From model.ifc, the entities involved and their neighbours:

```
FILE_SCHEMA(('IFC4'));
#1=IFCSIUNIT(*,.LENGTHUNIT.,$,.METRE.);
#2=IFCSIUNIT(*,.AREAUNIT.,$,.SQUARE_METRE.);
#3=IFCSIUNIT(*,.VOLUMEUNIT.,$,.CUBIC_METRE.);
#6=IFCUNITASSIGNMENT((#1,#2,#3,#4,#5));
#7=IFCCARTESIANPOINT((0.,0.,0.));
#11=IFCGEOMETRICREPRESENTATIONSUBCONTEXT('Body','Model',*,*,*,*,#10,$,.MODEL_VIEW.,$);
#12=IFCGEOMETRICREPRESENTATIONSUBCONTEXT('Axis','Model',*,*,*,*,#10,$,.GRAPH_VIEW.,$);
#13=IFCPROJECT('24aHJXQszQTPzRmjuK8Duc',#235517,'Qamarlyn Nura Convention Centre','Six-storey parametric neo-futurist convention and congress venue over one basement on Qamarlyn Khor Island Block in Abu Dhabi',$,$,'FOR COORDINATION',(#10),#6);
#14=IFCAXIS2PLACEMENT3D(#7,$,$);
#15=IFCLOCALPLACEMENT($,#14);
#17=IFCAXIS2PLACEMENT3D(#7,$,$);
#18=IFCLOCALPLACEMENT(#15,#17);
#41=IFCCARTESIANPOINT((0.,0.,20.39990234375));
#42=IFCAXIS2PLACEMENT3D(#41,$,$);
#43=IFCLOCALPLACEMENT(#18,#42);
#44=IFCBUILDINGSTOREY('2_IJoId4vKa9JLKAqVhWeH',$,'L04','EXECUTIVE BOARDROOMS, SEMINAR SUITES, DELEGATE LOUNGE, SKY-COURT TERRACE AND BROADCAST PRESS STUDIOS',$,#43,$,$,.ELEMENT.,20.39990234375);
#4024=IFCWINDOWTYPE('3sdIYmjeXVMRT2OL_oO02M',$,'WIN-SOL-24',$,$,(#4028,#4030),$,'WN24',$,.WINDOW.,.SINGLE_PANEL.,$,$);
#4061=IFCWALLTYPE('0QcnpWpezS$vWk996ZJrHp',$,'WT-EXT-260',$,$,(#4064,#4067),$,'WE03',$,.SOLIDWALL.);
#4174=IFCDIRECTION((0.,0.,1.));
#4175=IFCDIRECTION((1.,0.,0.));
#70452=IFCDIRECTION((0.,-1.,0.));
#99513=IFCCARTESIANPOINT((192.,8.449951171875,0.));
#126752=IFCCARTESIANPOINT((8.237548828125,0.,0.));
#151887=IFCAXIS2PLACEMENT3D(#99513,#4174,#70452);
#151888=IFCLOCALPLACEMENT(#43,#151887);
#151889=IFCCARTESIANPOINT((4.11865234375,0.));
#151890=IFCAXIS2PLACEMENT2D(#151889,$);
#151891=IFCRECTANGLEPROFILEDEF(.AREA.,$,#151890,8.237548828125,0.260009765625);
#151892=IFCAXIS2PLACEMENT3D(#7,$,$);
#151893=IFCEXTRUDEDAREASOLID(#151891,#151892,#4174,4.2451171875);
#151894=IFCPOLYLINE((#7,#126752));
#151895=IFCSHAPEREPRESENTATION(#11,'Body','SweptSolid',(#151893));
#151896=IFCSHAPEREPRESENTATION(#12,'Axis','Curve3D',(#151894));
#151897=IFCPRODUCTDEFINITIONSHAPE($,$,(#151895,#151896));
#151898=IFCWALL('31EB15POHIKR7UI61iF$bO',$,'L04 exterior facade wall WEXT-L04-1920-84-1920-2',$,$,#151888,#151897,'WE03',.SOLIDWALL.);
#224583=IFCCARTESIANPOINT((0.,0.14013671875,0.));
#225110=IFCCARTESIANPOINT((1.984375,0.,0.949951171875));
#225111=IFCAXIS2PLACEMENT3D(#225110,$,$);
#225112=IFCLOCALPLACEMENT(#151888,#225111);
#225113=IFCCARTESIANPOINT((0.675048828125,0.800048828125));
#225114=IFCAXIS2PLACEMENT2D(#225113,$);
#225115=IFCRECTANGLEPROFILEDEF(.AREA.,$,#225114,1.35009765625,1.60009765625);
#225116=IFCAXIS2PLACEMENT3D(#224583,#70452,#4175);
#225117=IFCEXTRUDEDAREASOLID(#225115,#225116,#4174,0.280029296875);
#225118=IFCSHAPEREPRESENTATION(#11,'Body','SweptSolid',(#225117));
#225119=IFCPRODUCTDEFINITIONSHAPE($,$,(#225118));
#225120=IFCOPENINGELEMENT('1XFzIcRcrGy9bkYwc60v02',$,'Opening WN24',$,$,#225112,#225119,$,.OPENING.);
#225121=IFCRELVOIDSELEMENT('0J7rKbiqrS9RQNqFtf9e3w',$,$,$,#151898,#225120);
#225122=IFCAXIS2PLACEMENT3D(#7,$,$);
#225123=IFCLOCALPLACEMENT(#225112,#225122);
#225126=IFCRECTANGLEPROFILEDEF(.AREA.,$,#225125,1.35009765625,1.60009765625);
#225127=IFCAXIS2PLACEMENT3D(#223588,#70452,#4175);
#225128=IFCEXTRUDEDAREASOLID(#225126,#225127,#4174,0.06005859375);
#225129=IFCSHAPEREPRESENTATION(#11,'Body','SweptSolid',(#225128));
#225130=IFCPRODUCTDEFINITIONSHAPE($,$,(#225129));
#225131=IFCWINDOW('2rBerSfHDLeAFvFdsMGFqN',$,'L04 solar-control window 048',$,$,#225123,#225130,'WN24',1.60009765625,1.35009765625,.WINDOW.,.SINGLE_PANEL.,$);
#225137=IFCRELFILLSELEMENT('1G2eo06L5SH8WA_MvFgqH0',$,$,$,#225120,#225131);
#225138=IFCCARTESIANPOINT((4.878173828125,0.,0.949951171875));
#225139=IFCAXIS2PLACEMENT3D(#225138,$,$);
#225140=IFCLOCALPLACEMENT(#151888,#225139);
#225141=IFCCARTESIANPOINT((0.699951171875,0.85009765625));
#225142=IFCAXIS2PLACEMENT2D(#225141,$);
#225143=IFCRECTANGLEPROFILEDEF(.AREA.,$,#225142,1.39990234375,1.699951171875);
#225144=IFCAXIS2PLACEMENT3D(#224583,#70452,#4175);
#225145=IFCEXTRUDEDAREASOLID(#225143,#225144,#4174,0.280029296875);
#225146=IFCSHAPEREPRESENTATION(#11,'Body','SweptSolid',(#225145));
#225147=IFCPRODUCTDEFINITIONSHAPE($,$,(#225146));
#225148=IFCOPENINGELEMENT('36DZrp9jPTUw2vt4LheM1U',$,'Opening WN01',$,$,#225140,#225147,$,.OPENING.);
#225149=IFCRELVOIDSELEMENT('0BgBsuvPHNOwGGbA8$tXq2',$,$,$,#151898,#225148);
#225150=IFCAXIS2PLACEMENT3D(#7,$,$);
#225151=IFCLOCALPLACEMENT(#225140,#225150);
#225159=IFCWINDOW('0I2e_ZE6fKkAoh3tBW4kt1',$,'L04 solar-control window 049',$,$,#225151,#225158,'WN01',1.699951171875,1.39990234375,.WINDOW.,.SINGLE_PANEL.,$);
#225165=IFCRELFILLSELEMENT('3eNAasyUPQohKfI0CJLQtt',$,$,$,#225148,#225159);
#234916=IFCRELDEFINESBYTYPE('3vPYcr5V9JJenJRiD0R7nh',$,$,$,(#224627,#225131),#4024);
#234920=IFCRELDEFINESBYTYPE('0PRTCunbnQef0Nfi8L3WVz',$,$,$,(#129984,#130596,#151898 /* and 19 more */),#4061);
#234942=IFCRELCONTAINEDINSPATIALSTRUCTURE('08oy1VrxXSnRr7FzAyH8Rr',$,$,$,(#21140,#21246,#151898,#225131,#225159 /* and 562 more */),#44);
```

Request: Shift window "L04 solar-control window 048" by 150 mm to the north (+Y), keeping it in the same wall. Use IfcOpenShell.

```python
import ifcopenshell
import ifcopenshell.api.geometry
import ifcopenshell.util.placement
import ifcopenshell.util.unit

model = ifcopenshell.open("model.ifc")
unit_scale = ifcopenshell.util.unit.calculate_unit_scale(model)

window = model.by_guid("2rBerSfHDLeAFvFdsMGFqN")
opening = window.FillsVoids[0].RelatingOpeningElement
wall = opening.VoidsElements[0].RelatingBuildingElement

wall_matrix = ifcopenshell.util.placement.get_local_placement(wall.ObjectPlacement)
shift = wall_matrix[:3, 0] * -0.15 / unit_scale
before = ifcopenshell.util.placement.get_local_placement(window.ObjectPlacement)[:3, 3].copy()

# The window is placed relative to its opening, so it follows when the opening moves.
matrix = ifcopenshell.util.placement.get_local_placement(opening.ObjectPlacement)
matrix[:3, 3] += shift
ifcopenshell.api.geometry.edit_object_placement(
    model, product=opening, matrix=matrix, is_si=False, should_transform_children=True
)

after = ifcopenshell.util.placement.get_local_placement(window.ObjectPlacement)[:3, 3]
print("window moved by", (after - before).round(3) + 0.0)

model.write("model_updated.ifc")
```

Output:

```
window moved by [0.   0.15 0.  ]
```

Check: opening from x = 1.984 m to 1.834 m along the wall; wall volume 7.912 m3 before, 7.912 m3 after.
